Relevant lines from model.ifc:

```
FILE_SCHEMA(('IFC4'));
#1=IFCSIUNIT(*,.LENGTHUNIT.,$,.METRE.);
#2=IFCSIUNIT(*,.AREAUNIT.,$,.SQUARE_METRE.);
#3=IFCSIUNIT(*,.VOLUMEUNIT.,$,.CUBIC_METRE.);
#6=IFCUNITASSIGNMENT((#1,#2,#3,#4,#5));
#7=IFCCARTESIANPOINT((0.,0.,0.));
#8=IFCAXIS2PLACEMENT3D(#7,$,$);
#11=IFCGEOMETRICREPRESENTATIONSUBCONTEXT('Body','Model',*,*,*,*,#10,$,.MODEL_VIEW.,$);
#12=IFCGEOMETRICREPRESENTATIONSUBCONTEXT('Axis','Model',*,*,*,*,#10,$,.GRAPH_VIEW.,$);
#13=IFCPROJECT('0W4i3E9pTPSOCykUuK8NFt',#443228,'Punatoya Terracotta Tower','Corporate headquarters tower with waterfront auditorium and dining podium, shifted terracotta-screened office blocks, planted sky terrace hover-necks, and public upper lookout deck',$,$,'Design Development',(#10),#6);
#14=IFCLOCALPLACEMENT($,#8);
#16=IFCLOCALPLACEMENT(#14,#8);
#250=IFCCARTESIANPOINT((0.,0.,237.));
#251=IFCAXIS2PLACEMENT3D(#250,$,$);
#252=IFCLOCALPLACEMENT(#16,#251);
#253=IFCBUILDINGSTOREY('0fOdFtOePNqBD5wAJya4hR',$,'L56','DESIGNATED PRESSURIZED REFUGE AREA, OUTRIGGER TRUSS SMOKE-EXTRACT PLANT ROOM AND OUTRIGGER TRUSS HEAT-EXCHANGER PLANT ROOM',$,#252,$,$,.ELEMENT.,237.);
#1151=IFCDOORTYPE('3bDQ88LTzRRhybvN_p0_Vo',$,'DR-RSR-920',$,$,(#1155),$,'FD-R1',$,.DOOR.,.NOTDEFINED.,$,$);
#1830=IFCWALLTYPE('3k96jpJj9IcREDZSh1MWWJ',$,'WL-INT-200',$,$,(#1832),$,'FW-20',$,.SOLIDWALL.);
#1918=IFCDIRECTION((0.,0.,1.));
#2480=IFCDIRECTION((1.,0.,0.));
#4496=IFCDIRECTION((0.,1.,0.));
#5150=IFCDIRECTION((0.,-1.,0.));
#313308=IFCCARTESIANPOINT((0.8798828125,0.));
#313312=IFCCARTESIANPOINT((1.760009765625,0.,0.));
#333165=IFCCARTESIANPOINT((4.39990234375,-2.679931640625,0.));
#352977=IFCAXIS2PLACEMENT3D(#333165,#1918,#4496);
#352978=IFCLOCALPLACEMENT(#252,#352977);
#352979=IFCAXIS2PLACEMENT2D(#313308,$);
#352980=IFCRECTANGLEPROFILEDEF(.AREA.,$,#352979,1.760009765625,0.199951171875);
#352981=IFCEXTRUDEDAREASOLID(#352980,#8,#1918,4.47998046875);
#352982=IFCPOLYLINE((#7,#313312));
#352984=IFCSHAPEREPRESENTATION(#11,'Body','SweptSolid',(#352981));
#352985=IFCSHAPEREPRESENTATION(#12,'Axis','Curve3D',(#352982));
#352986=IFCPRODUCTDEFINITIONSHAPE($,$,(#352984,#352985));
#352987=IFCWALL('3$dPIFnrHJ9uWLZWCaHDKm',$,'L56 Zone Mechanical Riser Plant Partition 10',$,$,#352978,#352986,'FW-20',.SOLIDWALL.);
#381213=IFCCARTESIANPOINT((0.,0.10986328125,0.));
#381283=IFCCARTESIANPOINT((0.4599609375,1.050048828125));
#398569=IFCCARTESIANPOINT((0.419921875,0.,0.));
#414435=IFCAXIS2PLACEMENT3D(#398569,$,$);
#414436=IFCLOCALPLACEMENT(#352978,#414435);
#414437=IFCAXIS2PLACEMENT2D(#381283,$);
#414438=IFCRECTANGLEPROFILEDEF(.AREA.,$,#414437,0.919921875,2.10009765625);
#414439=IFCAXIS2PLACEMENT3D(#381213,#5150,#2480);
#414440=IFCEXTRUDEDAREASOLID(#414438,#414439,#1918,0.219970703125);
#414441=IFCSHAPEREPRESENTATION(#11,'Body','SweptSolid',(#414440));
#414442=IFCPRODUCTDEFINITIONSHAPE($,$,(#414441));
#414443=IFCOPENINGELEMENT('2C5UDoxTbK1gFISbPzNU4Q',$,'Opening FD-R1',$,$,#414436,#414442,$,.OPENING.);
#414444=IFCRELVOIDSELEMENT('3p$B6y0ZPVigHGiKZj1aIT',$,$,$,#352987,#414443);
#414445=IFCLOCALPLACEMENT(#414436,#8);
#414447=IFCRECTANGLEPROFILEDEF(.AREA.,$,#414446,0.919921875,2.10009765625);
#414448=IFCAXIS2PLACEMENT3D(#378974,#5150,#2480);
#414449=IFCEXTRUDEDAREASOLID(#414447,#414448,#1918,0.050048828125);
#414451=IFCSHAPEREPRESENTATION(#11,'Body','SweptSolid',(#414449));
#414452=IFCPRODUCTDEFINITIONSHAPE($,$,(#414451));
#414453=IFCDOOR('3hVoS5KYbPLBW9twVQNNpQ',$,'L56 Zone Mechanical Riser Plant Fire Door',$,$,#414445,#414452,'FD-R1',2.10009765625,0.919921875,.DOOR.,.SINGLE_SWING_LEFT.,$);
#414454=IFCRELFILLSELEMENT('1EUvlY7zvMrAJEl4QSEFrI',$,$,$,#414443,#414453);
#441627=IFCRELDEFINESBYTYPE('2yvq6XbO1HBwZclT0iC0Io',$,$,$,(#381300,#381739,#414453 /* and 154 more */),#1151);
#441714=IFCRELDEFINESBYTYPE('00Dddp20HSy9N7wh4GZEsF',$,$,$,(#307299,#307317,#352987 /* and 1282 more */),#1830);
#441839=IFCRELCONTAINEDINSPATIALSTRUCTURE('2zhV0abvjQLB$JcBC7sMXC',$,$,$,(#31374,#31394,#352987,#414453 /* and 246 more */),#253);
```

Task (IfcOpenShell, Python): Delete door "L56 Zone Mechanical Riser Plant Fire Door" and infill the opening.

```python
import ifcopenshell
import ifcopenshell.api.feature
import ifcopenshell.api.root
import ifcopenshell.geom
import ifcopenshell.util.shape

model = ifcopenshell.open("model.ifc")
settings = ifcopenshell.geom.settings()


def volume(element):
    """Net volume in cubic metres, openings subtracted."""
    shape = ifcopenshell.geom.create_shape(settings, element)
    return ifcopenshell.util.shape.get_volume(shape.geometry)


door = model.by_guid("3hVoS5KYbPLBW9twVQNNpQ")
opening = door.FillsVoids[0].RelatingOpeningElement
wall = opening.VoidsElements[0].RelatingBuildingElement
before = volume(wall)

ifcopenshell.api.root.remove_product(model, product=door)
ifcopenshell.api.feature.remove_feature(model, feature=opening)

after = volume(wall)

print(f"wall volume {before:.3f} -> {after:.3f} m3")

model.write("model_updated.ifc")
```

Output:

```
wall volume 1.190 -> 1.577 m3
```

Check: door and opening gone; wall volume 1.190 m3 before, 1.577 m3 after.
